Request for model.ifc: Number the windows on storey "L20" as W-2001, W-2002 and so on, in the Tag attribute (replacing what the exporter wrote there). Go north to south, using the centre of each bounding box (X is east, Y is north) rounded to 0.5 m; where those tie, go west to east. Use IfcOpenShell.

First a look at what the model holds.

```python
import ifcopenshell
import ifcopenshell.util.element
import ifcopenshell.util.placement

model = ifcopenshell.open("model.ifc")
print(model.schema)
storey = next(s for s in model.by_type("IfcBuildingStorey") if s.Name == "L20")
windows = [e for e in ifcopenshell.util.element.get_decomposition(storey) if e.is_a("IfcWindow")]
for e in sorted(windows, key=lambda e: e.id()):
    origin = ifcopenshell.util.placement.get_local_placement(e.ObjectPlacement)[:3, 3]
    print(e.id(), e.Tag, e.Name, origin.round(2) + 0.0, sep=" | ")
```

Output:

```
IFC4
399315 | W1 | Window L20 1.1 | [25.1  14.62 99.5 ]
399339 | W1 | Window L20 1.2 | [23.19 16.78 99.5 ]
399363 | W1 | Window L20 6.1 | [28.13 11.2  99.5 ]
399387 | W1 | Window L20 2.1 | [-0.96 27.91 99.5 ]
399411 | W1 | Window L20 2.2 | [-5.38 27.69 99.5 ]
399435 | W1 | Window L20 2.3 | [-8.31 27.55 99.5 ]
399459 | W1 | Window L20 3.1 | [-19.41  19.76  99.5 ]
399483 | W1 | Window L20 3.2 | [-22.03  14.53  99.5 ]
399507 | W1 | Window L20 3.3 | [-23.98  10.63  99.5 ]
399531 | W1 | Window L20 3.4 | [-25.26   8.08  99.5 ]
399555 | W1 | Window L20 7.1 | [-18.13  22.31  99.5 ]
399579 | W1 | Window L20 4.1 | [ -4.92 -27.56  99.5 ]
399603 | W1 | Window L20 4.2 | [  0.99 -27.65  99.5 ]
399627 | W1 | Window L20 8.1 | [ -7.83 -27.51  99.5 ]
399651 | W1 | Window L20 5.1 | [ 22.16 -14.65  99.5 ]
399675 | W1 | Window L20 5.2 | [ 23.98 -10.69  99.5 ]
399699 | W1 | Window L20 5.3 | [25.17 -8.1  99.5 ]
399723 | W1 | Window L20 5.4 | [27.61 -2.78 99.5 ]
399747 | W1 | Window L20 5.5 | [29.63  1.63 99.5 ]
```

```python
import ifcopenshell
import ifcopenshell.geom
import ifcopenshell.util.element
import ifcopenshell.util.shape

model = ifcopenshell.open("model.ifc")
settings = ifcopenshell.geom.settings()
settings.set("use-world-coords", True)


def centre(element):
    shape = ifcopenshell.geom.create_shape(settings, element)
    return ifcopenshell.util.shape.get_bbox_centroid(shape.geometry)


storey = next(s for s in model.by_type("IfcBuildingStorey") if s.Name == "L20")
windows = [e for e in ifcopenshell.util.element.get_decomposition(storey) if e.is_a("IfcWindow")]

# Insertion points can sit at a corner or the storey origin, so sort by the geometry (in metres).
centres = {e: centre(e) for e in windows}
windows.sort(key=lambda e: (-round(centres[e][1] / 0.5), centres[e][0]))

for i, e in enumerate(windows, start=1):
    number = f"W-20{i:02d}"
    e.Tag = number
    print(e.id(), number)

model.write("model_v2.ifc")
```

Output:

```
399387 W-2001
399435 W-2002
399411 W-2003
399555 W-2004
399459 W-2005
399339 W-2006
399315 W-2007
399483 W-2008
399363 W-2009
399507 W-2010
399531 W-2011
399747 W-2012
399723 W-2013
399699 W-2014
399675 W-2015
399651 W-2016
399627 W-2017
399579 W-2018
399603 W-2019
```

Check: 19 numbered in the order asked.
